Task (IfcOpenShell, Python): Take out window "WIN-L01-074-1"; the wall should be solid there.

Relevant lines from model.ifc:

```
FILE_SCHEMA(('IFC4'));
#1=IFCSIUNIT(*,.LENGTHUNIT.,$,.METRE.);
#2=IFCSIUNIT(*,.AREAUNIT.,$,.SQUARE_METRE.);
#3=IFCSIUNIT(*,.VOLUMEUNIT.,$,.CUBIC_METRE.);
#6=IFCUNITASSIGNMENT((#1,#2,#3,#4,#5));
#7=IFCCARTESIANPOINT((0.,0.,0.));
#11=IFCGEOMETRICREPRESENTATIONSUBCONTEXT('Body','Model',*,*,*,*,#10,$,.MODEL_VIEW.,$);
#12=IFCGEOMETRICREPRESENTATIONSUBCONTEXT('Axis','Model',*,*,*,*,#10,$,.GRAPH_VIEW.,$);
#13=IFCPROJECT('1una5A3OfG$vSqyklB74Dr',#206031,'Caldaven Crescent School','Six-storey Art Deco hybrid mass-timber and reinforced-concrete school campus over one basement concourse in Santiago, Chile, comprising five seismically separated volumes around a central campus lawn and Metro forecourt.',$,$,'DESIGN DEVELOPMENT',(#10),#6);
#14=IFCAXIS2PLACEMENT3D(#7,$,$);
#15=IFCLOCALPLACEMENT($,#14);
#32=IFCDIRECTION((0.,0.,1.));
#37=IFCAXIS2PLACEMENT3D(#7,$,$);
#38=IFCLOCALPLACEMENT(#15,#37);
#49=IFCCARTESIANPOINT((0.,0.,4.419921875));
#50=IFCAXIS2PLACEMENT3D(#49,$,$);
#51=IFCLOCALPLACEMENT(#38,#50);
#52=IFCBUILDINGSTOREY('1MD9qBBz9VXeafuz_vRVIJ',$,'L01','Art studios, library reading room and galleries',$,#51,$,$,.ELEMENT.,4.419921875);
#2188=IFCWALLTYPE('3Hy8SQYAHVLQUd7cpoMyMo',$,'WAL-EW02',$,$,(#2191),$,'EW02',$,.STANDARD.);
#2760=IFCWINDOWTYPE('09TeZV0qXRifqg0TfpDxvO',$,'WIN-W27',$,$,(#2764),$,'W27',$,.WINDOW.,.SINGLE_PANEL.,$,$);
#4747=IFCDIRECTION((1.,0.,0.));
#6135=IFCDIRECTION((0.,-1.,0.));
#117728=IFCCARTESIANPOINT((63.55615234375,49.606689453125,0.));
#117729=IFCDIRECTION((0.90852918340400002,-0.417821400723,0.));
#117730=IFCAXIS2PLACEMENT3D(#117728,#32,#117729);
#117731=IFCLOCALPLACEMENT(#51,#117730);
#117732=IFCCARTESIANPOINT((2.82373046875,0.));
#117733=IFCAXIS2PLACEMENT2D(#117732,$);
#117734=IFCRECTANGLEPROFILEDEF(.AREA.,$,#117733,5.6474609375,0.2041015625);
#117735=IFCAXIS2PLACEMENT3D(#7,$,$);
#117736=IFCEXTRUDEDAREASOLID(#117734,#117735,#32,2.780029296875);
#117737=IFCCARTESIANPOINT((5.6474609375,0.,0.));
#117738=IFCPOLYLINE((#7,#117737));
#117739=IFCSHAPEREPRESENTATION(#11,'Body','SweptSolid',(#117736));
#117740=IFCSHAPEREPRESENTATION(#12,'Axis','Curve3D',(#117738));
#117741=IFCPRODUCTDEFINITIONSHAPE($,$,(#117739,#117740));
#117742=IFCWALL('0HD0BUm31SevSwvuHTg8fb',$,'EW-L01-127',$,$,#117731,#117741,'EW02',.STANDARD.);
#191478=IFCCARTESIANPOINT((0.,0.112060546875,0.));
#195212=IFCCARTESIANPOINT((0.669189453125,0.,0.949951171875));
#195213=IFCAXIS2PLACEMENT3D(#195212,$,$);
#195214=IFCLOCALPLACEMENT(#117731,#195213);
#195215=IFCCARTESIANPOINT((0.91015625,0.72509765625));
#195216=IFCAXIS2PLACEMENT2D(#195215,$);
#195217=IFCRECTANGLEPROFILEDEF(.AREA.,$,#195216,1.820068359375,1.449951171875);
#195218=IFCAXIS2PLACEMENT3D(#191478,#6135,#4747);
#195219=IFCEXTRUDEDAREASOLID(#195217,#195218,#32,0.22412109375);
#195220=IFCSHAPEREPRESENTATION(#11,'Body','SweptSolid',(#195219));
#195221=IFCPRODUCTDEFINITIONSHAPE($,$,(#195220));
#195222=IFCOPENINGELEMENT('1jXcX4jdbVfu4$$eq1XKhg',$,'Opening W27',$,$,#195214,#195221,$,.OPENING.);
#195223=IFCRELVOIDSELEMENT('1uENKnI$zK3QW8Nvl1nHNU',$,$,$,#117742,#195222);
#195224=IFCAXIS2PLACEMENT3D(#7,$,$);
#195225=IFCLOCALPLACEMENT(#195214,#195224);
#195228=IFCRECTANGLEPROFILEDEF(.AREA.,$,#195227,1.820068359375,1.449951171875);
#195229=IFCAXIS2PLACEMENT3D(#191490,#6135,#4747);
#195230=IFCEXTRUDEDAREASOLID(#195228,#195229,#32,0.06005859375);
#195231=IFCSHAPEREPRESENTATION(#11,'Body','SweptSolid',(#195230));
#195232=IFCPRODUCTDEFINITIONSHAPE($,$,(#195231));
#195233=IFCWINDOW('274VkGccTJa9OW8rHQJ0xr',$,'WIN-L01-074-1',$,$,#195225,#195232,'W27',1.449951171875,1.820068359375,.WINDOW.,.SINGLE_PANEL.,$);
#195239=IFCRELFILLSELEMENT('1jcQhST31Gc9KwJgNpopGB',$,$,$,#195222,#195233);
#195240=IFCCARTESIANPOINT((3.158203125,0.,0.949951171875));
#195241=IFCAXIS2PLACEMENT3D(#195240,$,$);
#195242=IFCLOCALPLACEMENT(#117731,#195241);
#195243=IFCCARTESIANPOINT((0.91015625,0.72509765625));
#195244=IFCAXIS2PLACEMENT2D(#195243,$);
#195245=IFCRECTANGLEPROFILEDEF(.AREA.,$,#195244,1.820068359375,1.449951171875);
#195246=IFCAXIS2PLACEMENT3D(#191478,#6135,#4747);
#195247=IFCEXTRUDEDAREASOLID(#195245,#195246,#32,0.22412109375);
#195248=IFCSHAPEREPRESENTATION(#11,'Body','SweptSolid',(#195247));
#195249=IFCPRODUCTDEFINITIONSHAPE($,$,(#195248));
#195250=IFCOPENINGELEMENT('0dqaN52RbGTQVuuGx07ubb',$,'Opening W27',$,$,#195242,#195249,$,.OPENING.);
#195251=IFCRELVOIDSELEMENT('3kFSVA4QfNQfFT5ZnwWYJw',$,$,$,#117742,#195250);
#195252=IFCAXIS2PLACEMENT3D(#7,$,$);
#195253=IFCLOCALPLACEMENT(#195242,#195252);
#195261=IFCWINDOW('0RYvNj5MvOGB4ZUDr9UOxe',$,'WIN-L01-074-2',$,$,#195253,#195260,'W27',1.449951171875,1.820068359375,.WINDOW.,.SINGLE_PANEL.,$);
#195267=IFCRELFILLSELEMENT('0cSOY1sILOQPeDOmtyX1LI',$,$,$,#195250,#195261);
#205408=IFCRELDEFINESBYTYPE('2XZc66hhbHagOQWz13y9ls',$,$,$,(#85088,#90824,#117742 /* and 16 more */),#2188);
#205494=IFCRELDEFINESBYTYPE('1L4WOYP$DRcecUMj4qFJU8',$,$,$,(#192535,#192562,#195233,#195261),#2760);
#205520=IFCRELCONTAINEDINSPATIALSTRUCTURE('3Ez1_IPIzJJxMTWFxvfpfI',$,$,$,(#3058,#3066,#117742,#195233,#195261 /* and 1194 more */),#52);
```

```python
import ifcopenshell
import ifcopenshell.api.feature
import ifcopenshell.api.root
import ifcopenshell.geom
import ifcopenshell.util.shape

model = ifcopenshell.open("model.ifc")
settings = ifcopenshell.geom.settings()


def volume(element):
    """Net volume in cubic metres, openings subtracted."""
    shape = ifcopenshell.geom.create_shape(settings, element)
    return ifcopenshell.util.shape.get_volume(shape.geometry)


window = model.by_guid("274VkGccTJa9OW8rHQJ0xr")
opening = window.FillsVoids[0].RelatingOpeningElement
wall = opening.VoidsElements[0].RelatingBuildingElement
before = volume(wall)

ifcopenshell.api.root.remove_product(model, product=window)
ifcopenshell.api.feature.remove_feature(model, feature=opening)

after = volume(wall)

print(f"wall volume {before:.3f} -> {after:.3f} m3")

model.write("model-out.ifc")
```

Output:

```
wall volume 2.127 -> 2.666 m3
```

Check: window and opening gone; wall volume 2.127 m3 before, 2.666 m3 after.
